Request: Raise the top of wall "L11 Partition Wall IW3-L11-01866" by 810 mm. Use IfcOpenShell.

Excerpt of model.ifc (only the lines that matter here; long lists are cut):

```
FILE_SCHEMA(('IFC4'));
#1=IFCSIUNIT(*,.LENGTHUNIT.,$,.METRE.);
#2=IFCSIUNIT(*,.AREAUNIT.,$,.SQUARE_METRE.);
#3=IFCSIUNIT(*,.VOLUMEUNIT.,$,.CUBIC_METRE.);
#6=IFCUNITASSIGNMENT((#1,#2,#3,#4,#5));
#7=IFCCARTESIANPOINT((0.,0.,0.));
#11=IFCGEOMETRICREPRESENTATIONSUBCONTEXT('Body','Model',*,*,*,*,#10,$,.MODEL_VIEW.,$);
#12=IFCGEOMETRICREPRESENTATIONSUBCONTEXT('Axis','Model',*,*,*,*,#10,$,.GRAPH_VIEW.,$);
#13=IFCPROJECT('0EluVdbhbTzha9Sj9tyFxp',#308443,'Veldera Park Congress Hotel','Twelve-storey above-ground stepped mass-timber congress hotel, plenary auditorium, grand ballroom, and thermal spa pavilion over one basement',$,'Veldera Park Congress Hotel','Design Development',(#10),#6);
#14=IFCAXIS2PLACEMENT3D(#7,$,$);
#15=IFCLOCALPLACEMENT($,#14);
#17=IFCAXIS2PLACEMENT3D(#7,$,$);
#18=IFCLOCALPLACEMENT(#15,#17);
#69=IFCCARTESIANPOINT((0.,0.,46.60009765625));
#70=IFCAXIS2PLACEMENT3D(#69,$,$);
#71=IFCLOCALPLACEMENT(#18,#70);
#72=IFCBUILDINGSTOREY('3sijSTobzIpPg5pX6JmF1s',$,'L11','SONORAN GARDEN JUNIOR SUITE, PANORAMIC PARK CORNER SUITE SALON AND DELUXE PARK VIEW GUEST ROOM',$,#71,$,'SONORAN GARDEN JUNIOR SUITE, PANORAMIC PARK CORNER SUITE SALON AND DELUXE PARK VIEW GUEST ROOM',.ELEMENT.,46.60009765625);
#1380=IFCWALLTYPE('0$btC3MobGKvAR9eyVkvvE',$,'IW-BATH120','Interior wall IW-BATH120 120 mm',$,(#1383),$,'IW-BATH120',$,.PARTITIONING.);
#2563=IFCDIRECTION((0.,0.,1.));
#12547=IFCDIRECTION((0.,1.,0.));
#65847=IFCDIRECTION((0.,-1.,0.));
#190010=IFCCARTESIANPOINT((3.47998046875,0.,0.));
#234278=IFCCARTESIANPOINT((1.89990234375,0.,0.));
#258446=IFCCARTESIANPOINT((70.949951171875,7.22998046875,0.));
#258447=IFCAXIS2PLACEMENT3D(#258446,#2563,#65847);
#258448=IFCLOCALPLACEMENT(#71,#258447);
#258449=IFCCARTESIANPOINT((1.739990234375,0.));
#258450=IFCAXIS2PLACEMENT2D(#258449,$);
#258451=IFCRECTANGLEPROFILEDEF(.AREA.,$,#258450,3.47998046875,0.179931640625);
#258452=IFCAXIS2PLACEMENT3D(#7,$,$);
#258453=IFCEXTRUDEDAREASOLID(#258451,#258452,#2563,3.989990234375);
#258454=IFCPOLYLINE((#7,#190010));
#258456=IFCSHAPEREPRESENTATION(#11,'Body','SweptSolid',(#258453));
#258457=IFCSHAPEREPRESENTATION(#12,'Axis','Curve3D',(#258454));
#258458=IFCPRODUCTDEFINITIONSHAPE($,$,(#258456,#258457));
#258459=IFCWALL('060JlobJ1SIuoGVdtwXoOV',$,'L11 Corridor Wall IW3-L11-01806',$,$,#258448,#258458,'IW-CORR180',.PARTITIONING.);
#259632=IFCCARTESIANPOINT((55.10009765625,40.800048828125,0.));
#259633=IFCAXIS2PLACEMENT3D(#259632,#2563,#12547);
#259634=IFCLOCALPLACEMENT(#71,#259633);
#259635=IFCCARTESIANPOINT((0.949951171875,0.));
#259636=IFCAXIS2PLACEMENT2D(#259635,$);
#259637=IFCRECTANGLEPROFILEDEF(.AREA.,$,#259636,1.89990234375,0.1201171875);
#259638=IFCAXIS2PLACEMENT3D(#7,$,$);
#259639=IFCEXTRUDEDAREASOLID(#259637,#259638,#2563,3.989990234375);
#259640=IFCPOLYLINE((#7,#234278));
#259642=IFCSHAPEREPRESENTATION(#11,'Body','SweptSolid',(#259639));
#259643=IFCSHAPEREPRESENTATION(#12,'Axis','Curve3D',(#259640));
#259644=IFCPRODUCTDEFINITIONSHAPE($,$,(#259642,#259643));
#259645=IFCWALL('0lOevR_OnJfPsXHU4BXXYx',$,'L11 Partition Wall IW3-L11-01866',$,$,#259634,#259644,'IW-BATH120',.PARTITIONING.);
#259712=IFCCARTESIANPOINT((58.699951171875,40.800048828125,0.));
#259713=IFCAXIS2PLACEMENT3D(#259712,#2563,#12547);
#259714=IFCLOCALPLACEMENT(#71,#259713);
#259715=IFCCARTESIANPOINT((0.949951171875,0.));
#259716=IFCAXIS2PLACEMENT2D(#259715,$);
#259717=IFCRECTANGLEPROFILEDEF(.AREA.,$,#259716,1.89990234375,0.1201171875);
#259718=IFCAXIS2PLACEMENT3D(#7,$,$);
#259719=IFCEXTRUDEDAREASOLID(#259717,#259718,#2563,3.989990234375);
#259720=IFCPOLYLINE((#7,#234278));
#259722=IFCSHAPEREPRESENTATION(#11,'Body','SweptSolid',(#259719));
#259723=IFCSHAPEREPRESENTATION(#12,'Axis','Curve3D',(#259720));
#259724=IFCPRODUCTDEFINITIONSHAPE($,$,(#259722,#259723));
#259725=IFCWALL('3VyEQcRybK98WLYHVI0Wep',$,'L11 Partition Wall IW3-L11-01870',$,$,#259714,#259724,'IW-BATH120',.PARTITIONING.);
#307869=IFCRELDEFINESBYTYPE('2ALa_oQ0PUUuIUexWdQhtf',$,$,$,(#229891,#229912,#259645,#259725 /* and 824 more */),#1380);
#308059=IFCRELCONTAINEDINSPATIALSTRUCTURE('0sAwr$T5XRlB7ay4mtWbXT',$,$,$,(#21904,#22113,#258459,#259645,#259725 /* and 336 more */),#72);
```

```python
import ifcopenshell
import ifcopenshell.geom
import ifcopenshell.util.representation
import ifcopenshell.util.shape
import ifcopenshell.util.unit

model = ifcopenshell.open("model.ifc")
unit_scale = ifcopenshell.util.unit.calculate_unit_scale(model)
settings = ifcopenshell.geom.settings()


def volume(element):
    """Net volume in cubic metres, openings subtracted."""
    shape = ifcopenshell.geom.create_shape(settings, element)
    return ifcopenshell.util.shape.get_volume(shape.geometry)


wall = model.by_guid("0lOevR_OnJfPsXHU4BXXYx")
before = volume(wall)

body = ifcopenshell.util.representation.get_representation(wall, "Model", "Body")
solid = body.Items[0]
old_height = solid.Depth
solid.Depth += 0.81 / unit_scale
after = volume(wall)

print(f"height {old_height:g} -> {solid.Depth:g}, volume {before:.3f} -> {after:.3f} m3")

model.write("model-out.ifc")
```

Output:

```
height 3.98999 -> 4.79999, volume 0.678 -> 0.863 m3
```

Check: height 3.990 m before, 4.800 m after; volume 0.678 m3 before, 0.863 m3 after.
